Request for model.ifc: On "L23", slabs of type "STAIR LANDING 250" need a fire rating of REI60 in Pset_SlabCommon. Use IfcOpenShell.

First a look at what the model holds.

```python
import ifcopenshell
import ifcopenshell.util.element

model = ifcopenshell.open("model.ifc")
print(model.schema)
storey = next(s for s in model.by_type("IfcBuildingStorey") if s.Name == "L23")
slabs = [e for e in ifcopenshell.util.element.get_decomposition(storey) if e.is_a("IfcSlab")]
seen = {}
for e in slabs:
    element_type = ifcopenshell.util.element.get_type(e)
    key = (element_type.Name if element_type != e and element_type else None, ifcopenshell.util.element.get_pset(e, "Pset_SlabCommon", "FireRating"))
    seen[key] = seen.get(key, 0) + 1
for (name, value), count in sorted(seen.items(), key=str):
    print(count, "x", name, "|", value)
```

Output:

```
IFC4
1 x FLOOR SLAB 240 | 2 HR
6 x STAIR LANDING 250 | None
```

```python
import ifcopenshell
import ifcopenshell.api.pset
import ifcopenshell.util.element

model = ifcopenshell.open("model.ifc")

storey = next(s for s in model.by_type("IfcBuildingStorey") if s.Name == "L23")
slabs = [e for e in ifcopenshell.util.element.get_decomposition(storey) if e.is_a("IfcSlab")]

count = 0
for e in slabs:
    element_type = ifcopenshell.util.element.get_type(e)
    if element_type in (None, e) or element_type.Name != "STAIR LANDING 250":
        continue
    # add_pset returns the element's existing set when there is one.
    pset = ifcopenshell.api.pset.add_pset(model, product=e, name="Pset_SlabCommon")
    ifcopenshell.api.pset.edit_pset(model, pset=pset, properties={"FireRating": "REI60"})
    count += 1

print(count, "slabs updated")

model.write("model_v2.ifc")
```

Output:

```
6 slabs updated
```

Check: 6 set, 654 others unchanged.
